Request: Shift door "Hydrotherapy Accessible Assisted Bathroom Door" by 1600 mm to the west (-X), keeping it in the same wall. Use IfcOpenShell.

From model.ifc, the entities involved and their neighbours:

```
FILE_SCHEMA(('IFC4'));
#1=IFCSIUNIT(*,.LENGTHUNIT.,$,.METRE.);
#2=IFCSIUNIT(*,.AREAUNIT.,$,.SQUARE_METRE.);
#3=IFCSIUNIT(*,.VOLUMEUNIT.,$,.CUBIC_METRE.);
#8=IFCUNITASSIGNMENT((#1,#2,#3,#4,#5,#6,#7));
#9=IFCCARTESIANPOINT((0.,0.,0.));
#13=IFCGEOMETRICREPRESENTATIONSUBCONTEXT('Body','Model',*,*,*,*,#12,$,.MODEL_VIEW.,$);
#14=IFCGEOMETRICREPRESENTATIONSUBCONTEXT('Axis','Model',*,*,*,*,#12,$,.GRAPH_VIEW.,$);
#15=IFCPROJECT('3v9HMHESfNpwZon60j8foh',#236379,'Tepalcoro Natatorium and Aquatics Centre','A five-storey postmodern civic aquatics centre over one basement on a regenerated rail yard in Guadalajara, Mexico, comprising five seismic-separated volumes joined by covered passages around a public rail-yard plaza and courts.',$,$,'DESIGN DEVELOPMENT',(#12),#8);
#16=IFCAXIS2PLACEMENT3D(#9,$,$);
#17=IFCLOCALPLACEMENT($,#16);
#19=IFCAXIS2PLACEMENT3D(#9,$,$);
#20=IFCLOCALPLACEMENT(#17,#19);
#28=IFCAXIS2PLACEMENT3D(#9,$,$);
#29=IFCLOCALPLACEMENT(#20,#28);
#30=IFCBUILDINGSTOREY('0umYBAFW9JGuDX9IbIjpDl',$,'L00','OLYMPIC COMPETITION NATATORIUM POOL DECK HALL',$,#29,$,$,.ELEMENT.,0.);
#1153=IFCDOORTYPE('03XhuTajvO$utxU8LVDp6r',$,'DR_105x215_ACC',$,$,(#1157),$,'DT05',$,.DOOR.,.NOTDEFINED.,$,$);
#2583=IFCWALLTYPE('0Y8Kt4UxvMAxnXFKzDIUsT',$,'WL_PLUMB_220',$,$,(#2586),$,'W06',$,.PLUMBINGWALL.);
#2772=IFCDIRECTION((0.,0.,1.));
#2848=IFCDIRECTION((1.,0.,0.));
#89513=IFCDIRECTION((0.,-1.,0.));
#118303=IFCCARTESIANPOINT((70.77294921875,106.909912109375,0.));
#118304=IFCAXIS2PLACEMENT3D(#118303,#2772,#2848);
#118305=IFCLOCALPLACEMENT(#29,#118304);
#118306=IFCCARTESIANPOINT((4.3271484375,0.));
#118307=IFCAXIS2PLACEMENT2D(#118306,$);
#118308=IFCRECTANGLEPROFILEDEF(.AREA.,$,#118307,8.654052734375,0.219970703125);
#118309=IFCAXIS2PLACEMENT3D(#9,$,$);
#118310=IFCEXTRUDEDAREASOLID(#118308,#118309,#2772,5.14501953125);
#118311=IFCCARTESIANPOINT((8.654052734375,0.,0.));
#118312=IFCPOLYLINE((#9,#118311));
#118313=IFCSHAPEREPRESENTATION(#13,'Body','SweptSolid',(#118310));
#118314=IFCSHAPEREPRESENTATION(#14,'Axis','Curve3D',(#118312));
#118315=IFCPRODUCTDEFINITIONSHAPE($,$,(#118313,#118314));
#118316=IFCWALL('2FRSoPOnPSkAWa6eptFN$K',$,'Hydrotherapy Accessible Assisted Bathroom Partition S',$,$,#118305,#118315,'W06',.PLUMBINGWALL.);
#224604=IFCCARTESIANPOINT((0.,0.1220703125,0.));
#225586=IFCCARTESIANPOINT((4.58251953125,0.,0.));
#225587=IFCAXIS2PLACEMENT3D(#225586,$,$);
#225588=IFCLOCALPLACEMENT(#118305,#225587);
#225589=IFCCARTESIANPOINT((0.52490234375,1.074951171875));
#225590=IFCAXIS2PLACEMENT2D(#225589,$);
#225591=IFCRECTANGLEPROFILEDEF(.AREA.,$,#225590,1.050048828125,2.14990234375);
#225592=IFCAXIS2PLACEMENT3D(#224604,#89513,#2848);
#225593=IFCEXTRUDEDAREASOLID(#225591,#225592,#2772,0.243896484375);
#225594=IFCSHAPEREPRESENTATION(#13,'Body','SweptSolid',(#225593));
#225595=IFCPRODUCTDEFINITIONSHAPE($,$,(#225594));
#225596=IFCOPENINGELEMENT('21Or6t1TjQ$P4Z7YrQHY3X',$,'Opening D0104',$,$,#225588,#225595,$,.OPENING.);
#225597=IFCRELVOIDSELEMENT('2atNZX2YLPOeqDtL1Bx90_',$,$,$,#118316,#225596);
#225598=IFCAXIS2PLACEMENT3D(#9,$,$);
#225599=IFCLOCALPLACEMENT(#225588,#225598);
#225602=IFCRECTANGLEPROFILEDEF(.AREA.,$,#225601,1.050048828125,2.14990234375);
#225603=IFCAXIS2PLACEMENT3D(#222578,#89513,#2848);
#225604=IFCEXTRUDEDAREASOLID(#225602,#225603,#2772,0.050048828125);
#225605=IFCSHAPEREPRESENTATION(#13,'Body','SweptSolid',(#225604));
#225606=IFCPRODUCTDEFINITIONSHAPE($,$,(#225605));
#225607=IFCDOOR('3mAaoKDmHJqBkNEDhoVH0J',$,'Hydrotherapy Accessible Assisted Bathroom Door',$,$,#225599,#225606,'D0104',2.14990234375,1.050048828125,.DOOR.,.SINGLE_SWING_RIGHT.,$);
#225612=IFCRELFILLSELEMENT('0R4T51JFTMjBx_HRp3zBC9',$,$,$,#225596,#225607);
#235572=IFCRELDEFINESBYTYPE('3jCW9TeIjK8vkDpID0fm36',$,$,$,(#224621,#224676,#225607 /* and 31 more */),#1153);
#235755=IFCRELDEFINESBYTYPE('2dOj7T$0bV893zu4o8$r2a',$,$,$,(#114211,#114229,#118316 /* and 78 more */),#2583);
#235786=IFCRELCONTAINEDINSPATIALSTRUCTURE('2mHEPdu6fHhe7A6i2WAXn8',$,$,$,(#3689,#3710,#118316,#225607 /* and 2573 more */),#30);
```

```python
import ifcopenshell
import ifcopenshell.api.geometry
import ifcopenshell.util.placement
import ifcopenshell.util.unit

model = ifcopenshell.open("model.ifc")
unit_scale = ifcopenshell.util.unit.calculate_unit_scale(model)

door = model.by_guid("3mAaoKDmHJqBkNEDhoVH0J")
opening = door.FillsVoids[0].RelatingOpeningElement
wall = opening.VoidsElements[0].RelatingBuildingElement

wall_matrix = ifcopenshell.util.placement.get_local_placement(wall.ObjectPlacement)
shift = wall_matrix[:3, 0] * -1.6 / unit_scale
before = ifcopenshell.util.placement.get_local_placement(door.ObjectPlacement)[:3, 3].copy()

# The door is placed relative to its opening, so it follows when the opening moves.
matrix = ifcopenshell.util.placement.get_local_placement(opening.ObjectPlacement)
matrix[:3, 3] += shift
ifcopenshell.api.geometry.edit_object_placement(
    model, product=opening, matrix=matrix, is_si=False, should_transform_children=True
)

after = ifcopenshell.util.placement.get_local_placement(door.ObjectPlacement)[:3, 3]
print("door moved by", (after - before).round(3) + 0.0)

model.write("model_rev.ifc")
```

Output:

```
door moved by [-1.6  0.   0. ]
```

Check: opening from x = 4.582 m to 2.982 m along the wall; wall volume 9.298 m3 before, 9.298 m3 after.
